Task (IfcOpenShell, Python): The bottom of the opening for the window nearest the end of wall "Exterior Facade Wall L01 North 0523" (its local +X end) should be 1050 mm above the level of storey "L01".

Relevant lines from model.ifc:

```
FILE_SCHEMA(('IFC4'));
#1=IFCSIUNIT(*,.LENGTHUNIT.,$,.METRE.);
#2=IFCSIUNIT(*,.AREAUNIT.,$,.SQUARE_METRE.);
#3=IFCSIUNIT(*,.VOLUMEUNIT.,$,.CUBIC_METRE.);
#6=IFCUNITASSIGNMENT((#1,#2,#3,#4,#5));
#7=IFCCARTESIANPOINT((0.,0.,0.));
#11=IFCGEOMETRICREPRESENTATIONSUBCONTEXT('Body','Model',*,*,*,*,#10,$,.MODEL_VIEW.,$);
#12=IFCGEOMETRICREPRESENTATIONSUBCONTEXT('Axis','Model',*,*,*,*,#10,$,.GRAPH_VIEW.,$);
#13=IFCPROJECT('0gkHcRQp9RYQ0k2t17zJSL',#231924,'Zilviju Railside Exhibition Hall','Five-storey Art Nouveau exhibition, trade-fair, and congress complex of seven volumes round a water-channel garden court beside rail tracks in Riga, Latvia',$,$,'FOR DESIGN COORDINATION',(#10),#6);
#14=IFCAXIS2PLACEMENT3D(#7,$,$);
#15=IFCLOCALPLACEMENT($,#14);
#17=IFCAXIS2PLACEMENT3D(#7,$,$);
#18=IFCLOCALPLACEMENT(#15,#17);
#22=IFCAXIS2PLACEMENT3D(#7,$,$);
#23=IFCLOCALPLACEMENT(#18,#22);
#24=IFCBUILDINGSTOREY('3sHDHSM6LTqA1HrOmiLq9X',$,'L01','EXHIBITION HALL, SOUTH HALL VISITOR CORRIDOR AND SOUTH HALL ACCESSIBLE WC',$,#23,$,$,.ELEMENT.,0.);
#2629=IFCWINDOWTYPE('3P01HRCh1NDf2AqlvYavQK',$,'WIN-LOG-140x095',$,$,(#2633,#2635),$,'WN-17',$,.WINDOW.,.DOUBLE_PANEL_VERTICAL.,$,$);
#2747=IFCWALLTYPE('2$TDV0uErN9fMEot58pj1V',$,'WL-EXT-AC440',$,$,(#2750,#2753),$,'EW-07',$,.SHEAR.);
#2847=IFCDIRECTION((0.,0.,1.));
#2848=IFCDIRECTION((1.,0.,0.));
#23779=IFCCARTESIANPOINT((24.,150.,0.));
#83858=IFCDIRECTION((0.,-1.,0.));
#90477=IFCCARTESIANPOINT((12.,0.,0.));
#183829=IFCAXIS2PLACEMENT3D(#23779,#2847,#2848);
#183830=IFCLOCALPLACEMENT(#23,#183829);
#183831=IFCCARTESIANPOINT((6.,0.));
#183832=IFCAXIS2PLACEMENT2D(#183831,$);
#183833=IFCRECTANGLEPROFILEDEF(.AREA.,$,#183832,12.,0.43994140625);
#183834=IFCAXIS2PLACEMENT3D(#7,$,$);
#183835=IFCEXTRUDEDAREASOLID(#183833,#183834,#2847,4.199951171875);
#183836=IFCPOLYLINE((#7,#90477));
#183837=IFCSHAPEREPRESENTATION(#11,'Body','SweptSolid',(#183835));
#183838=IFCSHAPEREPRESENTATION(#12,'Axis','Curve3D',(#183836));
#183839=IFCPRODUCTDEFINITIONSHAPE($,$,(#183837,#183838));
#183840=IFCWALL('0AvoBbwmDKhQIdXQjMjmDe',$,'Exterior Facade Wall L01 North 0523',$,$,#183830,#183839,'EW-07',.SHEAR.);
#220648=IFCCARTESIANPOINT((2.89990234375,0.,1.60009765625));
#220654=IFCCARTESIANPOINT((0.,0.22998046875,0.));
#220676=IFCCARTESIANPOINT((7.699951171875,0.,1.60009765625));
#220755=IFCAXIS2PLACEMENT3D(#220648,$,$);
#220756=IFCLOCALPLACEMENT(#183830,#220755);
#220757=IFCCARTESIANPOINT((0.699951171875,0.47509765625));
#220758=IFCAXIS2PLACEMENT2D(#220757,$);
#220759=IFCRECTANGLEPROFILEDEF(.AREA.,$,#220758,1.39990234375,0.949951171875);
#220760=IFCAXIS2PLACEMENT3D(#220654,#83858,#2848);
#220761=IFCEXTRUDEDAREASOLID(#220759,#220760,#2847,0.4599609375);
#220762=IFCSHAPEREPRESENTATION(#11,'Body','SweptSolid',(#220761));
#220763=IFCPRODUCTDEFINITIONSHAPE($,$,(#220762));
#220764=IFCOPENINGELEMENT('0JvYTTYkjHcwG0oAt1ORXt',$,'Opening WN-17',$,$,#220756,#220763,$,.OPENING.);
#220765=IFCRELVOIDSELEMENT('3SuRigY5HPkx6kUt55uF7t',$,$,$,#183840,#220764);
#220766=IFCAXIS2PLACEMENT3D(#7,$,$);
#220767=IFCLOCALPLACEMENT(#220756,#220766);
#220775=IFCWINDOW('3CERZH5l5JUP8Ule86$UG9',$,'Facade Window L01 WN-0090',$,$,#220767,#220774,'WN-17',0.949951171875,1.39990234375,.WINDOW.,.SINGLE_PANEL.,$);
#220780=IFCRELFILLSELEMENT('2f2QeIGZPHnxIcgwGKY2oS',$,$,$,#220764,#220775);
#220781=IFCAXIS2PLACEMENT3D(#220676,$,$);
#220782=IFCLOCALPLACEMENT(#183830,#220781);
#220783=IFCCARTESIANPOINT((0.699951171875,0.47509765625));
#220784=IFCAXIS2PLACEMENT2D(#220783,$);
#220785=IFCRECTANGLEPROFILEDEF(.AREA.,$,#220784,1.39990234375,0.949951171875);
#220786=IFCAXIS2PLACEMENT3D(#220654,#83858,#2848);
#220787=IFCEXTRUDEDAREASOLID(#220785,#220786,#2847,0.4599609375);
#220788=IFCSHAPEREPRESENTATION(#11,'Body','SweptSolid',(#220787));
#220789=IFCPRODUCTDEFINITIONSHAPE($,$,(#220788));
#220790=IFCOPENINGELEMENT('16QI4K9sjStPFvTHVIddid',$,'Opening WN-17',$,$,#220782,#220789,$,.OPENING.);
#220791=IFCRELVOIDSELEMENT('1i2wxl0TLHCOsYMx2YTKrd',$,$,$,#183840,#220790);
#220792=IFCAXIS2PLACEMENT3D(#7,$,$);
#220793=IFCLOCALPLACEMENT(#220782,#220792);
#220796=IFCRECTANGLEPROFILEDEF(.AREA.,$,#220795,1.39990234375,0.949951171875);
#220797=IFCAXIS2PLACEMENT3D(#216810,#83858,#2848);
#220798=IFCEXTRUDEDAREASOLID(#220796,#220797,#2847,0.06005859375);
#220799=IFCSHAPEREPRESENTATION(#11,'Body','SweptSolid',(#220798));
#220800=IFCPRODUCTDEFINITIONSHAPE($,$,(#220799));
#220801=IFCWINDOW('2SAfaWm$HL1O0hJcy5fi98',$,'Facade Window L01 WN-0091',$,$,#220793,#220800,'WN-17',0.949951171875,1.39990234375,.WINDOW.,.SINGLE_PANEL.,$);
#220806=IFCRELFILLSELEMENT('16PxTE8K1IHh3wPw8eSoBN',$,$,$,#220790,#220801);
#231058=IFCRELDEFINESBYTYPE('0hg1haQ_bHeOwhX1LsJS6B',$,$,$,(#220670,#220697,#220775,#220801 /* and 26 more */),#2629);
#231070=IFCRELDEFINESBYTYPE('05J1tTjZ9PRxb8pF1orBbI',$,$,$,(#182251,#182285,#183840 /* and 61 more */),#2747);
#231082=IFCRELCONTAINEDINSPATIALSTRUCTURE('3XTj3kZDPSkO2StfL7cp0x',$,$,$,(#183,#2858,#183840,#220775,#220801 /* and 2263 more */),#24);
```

```python
import numpy as np
import ifcopenshell
import ifcopenshell.api.geometry
import ifcopenshell.geom
import ifcopenshell.util.element
import ifcopenshell.util.placement
import ifcopenshell.util.shape
import ifcopenshell.util.unit

model = ifcopenshell.open("model.ifc")
unit_scale = ifcopenshell.util.unit.calculate_unit_scale(model)

window = model.by_guid("2SAfaWm$HL1O0hJcy5fi98")
opening = window.FillsVoids[0].RelatingOpeningElement
storey = ifcopenshell.util.element.get_container(window, ifc_class="IfcBuildingStorey")
level = ifcopenshell.util.placement.get_local_placement(storey.ObjectPlacement)[2, 3]

# The opening's origin need not be at the sill, so measure its lowest point.
shape = ifcopenshell.geom.create_shape(ifcopenshell.geom.settings(), opening)
bottom = ifcopenshell.util.shape.get_shape_bottom_elevation(shape, shape.geometry) / unit_scale
dz = level + 1.05 / unit_scale - bottom

shift = np.array([0.0, 0.0, dz])
# The window is placed relative to its opening, so it follows when the opening moves.
matrix = ifcopenshell.util.placement.get_local_placement(opening.ObjectPlacement)
matrix[:3, 3] += shift
ifcopenshell.api.geometry.edit_object_placement(
    model, product=opening, matrix=matrix, is_si=False, should_transform_children=True
)

print(f"moved by {dz * unit_scale:+.3f} m")

model.write("model_updated.ifc")
```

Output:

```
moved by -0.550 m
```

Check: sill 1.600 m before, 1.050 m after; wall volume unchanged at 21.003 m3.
